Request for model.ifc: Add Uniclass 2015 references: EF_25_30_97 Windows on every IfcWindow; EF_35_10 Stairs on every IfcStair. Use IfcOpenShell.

First a look at what the model holds.

```python
import ifcopenshell

model = ifcopenshell.open("model.ifc")
print(model.schema)
print("classifications:", [c.Name for c in model.by_type("IfcClassification")])
for ifc_class in ("IfcDoor", "IfcRoof", "IfcStair", "IfcWall", "IfcWindow"):
    print(ifc_class, len(model.by_type(ifc_class)))
```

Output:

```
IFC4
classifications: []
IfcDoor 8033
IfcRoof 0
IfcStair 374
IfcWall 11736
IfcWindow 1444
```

```python
import ifcopenshell
import ifcopenshell.api.classification

model = ifcopenshell.open("model.ifc")

system = ifcopenshell.api.classification.add_classification(model, classification="Uniclass 2015")

codes = {
    "IfcWindow": ("EF_25_30_97", "Windows"),
    "IfcStair": ("EF_35_10", "Stairs"),
}
for ifc_class, (code, name) in codes.items():
    products = model.by_type(ifc_class)
    ifcopenshell.api.classification.add_reference(
        model, products=products, classification=system, identification=code, name=name
    )
    print(code, len(products))

model.write("model_updated.ifc")
```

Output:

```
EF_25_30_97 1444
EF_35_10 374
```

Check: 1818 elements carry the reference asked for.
